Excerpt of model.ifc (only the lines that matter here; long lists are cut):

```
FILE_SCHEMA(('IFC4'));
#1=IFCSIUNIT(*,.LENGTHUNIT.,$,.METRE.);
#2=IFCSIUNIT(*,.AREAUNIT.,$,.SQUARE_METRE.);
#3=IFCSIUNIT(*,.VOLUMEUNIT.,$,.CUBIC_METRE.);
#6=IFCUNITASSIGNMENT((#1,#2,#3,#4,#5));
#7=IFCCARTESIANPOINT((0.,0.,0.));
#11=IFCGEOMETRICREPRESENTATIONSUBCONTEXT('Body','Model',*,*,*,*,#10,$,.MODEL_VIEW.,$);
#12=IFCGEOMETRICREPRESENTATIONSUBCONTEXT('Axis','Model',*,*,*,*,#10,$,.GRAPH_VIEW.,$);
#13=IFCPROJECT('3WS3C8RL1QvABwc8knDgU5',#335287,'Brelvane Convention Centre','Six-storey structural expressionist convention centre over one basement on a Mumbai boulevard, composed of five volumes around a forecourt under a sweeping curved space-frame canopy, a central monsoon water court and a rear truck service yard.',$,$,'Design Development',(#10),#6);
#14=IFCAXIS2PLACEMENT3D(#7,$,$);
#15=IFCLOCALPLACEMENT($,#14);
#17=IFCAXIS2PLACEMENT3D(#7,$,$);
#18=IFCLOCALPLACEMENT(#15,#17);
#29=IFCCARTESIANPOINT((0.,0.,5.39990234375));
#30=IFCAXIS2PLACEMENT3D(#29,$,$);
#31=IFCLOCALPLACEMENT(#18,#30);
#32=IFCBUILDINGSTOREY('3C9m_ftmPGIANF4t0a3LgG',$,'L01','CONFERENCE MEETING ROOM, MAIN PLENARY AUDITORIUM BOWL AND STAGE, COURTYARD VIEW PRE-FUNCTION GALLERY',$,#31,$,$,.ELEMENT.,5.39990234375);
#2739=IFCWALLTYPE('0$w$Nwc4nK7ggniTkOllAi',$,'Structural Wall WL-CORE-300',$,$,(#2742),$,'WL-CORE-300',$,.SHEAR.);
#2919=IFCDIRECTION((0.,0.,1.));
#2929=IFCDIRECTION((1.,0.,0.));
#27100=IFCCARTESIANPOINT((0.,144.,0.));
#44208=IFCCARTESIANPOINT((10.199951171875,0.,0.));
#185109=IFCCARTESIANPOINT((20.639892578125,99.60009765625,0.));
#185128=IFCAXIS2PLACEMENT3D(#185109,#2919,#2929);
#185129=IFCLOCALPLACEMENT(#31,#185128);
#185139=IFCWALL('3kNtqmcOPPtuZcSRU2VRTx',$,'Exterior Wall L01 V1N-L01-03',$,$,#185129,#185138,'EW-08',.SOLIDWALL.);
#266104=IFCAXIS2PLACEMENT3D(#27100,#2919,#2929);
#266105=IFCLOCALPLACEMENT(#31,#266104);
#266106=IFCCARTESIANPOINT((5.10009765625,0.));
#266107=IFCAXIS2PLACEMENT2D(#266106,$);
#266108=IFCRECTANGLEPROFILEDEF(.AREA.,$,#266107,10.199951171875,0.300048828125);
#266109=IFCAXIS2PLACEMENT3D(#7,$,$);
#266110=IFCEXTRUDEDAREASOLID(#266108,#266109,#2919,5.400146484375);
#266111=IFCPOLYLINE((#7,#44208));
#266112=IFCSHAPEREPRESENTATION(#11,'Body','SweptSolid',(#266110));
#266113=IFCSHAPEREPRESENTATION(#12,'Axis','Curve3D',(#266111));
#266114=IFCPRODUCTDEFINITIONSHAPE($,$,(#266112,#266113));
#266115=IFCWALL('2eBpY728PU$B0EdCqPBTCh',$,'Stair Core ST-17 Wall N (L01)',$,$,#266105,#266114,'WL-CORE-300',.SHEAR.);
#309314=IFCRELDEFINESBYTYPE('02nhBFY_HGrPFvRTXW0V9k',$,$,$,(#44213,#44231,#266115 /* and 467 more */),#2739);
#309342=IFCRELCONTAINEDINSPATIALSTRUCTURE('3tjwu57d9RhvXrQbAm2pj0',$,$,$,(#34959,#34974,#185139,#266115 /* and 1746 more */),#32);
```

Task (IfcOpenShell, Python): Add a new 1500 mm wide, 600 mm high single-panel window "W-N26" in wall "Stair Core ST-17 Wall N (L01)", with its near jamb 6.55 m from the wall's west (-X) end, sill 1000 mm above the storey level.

```python
import numpy as np
import ifcopenshell
import ifcopenshell.api.feature
import ifcopenshell.api.geometry
import ifcopenshell.api.root
import ifcopenshell.api.spatial
import ifcopenshell.geom
import ifcopenshell.util.element
import ifcopenshell.util.placement
import ifcopenshell.util.representation
import ifcopenshell.util.shape
import ifcopenshell.util.unit

model = ifcopenshell.open("model.ifc")
unit_scale = ifcopenshell.util.unit.calculate_unit_scale(model)
settings = ifcopenshell.geom.settings()


def volume(element):
    """Net volume in cubic metres, openings subtracted."""
    shape = ifcopenshell.geom.create_shape(settings, element)
    return ifcopenshell.util.shape.get_volume(shape.geometry)


wall = model.by_id(266115)
storey = ifcopenshell.util.element.get_container(wall, ifc_class="IfcBuildingStorey")
context = ifcopenshell.util.representation.get_context(model, "Model", "Body", "MODEL_VIEW")
before = volume(wall)

width, height, from_end, sill = 1.5, 0.6, 6.55, 1  # metres

# The wall runs along its own X axis, and the end named is its -X end.
wall_shape = ifcopenshell.geom.create_shape(settings, wall)
x, y, z = ifcopenshell.util.shape.get_vertices(wall_shape.geometry).T
start = x.min() + from_end
face, thickness = float(y.min()), float(y.max() - y.min())
wall_matrix = ifcopenshell.util.placement.get_local_placement(wall.ObjectPlacement)
level = ifcopenshell.util.placement.get_local_placement(storey.ObjectPlacement)[2, 3]


def in_wall(x, y):
    """Placement at x, y metres in the wall's axes, at sill height."""
    matrix = wall_matrix.copy()
    matrix[:, 3] = wall_matrix @ np.array([x / unit_scale, y / unit_scale, 0.0, 1.0])
    matrix[2, 3] = level + sill / unit_scale
    return matrix


# Opening: a box that overshoots both wall faces by 50 mm.
opening = ifcopenshell.api.root.create_entity(model, ifc_class="IfcOpeningElement", predefined_type="OPENING")
box = ifcopenshell.api.geometry.add_wall_representation(
    model, context=context, length=width, height=height, thickness=thickness + 0.1
)
ifcopenshell.api.geometry.assign_representation(model, product=opening, representation=box)
ifcopenshell.api.geometry.edit_object_placement(model, product=opening, matrix=in_wall(start, face - 0.05), is_si=False)
ifcopenshell.api.feature.add_feature(model, feature=opening, element=wall)

window = ifcopenshell.api.root.create_entity(model, ifc_class="IfcWindow", name="W-N26", predefined_type="WINDOW")
window.OverallWidth, window.OverallHeight = width / unit_scale, height / unit_scale
window.PartitioningType = "SINGLE_PANEL"
body = ifcopenshell.api.geometry.add_window_representation(
    model,
    context=context,
    overall_width=window.OverallWidth,
    overall_height=window.OverallHeight,
    partition_type="SINGLE_PANEL",
)
ifcopenshell.api.geometry.assign_representation(model, product=window, representation=body)
ifcopenshell.api.spatial.assign_container(model, products=[window], relating_structure=storey)
ifcopenshell.api.feature.add_filling(model, opening=opening, element=window)

# Centre the window in the wall's thickness.
ifcopenshell.api.geometry.edit_object_placement(model, product=window, matrix=in_wall(start, face), is_si=False)
window_shape = ifcopenshell.geom.create_shape(settings, window)
depth = ifcopenshell.util.shape.get_vertices(window_shape.geometry)[:, 1]
offset = face + thickness / 2 - (depth.min() + depth.max()) / 2
ifcopenshell.api.geometry.edit_object_placement(model, product=window, matrix=in_wall(start, offset), is_si=False)

after = volume(wall)

print(f"wall volume {before:.3f} -> {after:.3f} m3")

model.write("model_edited.ifc")
```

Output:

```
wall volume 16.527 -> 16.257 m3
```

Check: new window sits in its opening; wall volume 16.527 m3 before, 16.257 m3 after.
